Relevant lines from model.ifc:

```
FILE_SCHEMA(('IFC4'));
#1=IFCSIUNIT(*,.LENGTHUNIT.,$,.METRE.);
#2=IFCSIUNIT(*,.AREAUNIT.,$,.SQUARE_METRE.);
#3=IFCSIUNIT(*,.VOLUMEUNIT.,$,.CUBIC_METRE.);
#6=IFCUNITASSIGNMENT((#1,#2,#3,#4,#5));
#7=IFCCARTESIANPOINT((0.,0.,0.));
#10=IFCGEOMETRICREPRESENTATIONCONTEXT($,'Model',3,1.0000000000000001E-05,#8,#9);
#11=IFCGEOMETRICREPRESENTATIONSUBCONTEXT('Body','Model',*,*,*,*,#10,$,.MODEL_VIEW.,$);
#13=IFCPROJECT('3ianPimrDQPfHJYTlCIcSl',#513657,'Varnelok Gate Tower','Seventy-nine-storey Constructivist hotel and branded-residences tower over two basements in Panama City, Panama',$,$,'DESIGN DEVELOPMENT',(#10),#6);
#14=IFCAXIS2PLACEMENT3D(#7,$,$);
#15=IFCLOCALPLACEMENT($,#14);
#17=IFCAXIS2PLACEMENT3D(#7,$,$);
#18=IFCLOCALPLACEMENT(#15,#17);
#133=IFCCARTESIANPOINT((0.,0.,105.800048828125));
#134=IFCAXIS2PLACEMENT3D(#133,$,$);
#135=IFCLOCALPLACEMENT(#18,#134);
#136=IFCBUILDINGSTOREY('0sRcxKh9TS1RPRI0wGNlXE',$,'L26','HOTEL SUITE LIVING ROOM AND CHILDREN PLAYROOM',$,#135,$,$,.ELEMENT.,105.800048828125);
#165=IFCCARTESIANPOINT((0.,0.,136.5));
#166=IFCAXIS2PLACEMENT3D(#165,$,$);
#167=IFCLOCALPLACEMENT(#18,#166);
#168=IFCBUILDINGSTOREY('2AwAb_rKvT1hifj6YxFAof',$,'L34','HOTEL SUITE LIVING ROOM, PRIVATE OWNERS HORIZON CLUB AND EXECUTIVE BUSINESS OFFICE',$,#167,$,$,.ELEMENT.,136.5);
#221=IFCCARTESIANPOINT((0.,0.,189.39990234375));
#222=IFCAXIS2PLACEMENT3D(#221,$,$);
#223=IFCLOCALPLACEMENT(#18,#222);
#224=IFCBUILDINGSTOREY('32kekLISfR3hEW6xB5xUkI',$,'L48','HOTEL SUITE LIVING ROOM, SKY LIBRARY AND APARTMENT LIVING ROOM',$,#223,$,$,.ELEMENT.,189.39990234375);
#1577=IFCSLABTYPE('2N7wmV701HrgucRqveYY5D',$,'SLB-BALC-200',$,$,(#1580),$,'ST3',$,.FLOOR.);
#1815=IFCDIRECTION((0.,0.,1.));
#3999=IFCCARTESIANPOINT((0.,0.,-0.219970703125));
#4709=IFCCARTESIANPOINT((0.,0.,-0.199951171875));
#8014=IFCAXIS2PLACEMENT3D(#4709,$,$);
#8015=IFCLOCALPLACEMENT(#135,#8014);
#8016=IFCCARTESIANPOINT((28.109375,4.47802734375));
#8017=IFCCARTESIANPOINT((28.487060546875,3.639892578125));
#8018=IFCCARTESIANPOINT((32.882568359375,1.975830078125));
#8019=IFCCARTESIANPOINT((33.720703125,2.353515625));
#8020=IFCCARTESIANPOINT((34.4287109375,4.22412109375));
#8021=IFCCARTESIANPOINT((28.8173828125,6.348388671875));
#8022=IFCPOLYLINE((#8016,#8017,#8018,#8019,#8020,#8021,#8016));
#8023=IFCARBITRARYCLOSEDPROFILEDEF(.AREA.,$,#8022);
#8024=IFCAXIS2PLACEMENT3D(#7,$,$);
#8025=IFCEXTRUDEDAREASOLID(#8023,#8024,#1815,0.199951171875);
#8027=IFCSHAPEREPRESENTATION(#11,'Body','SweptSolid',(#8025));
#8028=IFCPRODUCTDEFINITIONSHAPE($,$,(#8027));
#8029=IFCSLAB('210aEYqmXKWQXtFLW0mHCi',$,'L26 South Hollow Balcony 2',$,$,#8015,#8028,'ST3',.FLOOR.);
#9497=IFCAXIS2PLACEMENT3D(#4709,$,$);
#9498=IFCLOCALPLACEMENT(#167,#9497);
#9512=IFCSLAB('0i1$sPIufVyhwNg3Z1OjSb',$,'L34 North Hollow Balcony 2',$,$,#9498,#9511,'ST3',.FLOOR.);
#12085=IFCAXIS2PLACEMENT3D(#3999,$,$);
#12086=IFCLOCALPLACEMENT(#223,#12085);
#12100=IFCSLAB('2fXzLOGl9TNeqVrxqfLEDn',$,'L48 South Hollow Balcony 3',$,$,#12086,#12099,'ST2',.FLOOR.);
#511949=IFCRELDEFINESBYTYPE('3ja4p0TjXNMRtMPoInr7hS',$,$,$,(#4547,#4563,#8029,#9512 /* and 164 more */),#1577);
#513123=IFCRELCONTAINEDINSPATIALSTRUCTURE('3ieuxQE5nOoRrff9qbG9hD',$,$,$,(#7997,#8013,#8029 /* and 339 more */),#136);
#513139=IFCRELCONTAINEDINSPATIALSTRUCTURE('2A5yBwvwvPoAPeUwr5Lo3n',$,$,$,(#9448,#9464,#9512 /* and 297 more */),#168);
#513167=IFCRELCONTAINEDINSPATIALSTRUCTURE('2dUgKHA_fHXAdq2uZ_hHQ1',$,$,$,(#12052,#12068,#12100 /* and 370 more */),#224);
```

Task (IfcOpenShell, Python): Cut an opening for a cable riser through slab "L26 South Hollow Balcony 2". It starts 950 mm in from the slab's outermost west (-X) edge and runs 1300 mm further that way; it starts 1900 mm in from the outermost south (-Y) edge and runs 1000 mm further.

```python
import numpy as np
import ifcopenshell
import ifcopenshell.api.feature
import ifcopenshell.api.geometry
import ifcopenshell.api.root
import ifcopenshell.geom
import ifcopenshell.util.placement
import ifcopenshell.util.representation
import ifcopenshell.util.shape
import ifcopenshell.util.unit

model = ifcopenshell.open("model.ifc")
unit_scale = ifcopenshell.util.unit.calculate_unit_scale(model)
settings = ifcopenshell.geom.settings()


def volume(element):
    """Net volume in cubic metres, openings subtracted."""
    shape = ifcopenshell.geom.create_shape(settings, element)
    return ifcopenshell.util.shape.get_volume(shape.geometry)


slab = model.by_guid("210aEYqmXKWQXtFLW0mHCi")
before = volume(slab)

# Extent in the slab's own axes, in metres. The edges named are its -X and -Y sides.
slab_shape = ifcopenshell.geom.create_shape(settings, slab)
vertices = ifcopenshell.util.shape.get_vertices(slab_shape.geometry)
x_min, y_min, bottom = vertices.min(axis=0)
top = vertices[:, 2].max()

opening = ifcopenshell.api.root.create_entity(model, ifc_class="IfcOpeningElement", name="Cable riser opening", predefined_type="OPENING")
context = ifcopenshell.util.representation.get_context(model, "Model", "Body", "MODEL_VIEW")
width, depth = 1.3, 1
outline = [(0.0, 0.0), (width, 0.0), (width, depth), (0.0, depth), (0.0, 0.0)]
# Overshoot both faces by 50 mm so the cut is clean.
shape = ifcopenshell.api.geometry.add_slab_representation(
    model, context=context, depth=top - bottom + 0.1, polyline=outline
)
ifcopenshell.api.geometry.assign_representation(model, product=opening, representation=shape)

matrix = ifcopenshell.util.placement.get_local_placement(slab.ObjectPlacement)
matrix[:, 3] = matrix @ np.append(np.array([x_min + 0.95, y_min + 1.9, bottom - 0.05]) / unit_scale, 1.0)
ifcopenshell.api.geometry.edit_object_placement(model, product=opening, matrix=matrix, is_si=False)
ifcopenshell.api.feature.add_feature(model, feature=opening, element=slab)

after = volume(slab)

print(f"slab volume {before:.3f} -> {after:.3f} m3")

model.write("model_edited.ifc")
```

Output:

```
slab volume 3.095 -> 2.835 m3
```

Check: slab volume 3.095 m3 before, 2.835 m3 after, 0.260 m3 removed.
